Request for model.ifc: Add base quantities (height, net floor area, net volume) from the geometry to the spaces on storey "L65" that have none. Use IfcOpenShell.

First a look at what the model holds.

```python
import ifcopenshell
import ifcopenshell.util.element
import ifcopenshell.util.unit

model = ifcopenshell.open("model.ifc")
print(model.schema)
for unit_type in ("LENGTHUNIT", "AREAUNIT", "VOLUMEUNIT"):
    print(unit_type, ifcopenshell.util.unit.calculate_unit_scale(model, unit_type))
storey = next(s for s in model.by_type("IfcBuildingStorey") if s.Name == "L65")
spaces = [e for e in ifcopenshell.util.element.get_decomposition(storey) if e.is_a("IfcSpace")]
for e in sorted(spaces, key=lambda e: e.id()):
    print(e.id(), e.is_a(), e.Name, list(ifcopenshell.util.element.get_psets(e, qtos_only=True)), sep=" | ")
```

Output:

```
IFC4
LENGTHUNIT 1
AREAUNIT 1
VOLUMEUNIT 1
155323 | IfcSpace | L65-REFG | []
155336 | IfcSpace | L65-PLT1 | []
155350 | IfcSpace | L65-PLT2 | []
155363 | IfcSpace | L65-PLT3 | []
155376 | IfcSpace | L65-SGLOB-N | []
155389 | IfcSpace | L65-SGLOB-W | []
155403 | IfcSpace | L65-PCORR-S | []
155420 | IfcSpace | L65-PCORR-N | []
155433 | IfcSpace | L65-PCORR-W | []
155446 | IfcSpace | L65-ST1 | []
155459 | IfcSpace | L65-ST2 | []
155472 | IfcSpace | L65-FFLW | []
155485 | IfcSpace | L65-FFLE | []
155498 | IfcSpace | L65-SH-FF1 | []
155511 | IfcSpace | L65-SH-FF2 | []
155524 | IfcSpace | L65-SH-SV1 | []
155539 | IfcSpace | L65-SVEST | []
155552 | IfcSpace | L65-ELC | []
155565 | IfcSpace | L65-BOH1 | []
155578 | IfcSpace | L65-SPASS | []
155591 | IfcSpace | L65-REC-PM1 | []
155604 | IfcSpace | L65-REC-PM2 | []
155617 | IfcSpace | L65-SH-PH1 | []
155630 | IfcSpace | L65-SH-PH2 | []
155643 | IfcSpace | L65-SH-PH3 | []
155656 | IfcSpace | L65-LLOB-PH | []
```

```python
import ifcopenshell
import ifcopenshell.api.pset
import ifcopenshell.geom
import ifcopenshell.util.element
import ifcopenshell.util.shape
import ifcopenshell.util.unit

model = ifcopenshell.open("model.ifc")
unit_scale = ifcopenshell.util.unit.calculate_unit_scale(model)
area_scale = ifcopenshell.util.unit.calculate_unit_scale(model, "AREAUNIT")
volume_scale = ifcopenshell.util.unit.calculate_unit_scale(model, "VOLUMEUNIT")
settings = ifcopenshell.geom.settings()

storey = next(s for s in model.by_type("IfcBuildingStorey") if s.Name == "L65")
spaces = [e for e in ifcopenshell.util.element.get_decomposition(storey) if e.is_a("IfcSpace")]

for e in sorted(spaces, key=lambda e: e.id()):
    if ifcopenshell.util.element.get_psets(e, qtos_only=True, should_inherit=False):
        continue
    # Geometry comes back in metres, in the element's own axes.
    shape = ifcopenshell.geom.create_shape(settings, e)
    values = {
        "Height": ifcopenshell.util.shape.get_z(shape.geometry) / unit_scale,
        "NetFloorArea": ifcopenshell.util.shape.get_footprint_area(shape.geometry) / area_scale,
        "NetVolume": ifcopenshell.util.shape.get_volume(shape.geometry) / volume_scale,
    }
    qto = ifcopenshell.api.pset.add_qto(model, product=e, name="Qto_SpaceBaseQuantities")
    ifcopenshell.api.pset.edit_qto(model, qto=qto, properties=values)
    print(e.id(), {k: round(v, 3) for k, v in values.items()})

model.write("model-out.ifc")
```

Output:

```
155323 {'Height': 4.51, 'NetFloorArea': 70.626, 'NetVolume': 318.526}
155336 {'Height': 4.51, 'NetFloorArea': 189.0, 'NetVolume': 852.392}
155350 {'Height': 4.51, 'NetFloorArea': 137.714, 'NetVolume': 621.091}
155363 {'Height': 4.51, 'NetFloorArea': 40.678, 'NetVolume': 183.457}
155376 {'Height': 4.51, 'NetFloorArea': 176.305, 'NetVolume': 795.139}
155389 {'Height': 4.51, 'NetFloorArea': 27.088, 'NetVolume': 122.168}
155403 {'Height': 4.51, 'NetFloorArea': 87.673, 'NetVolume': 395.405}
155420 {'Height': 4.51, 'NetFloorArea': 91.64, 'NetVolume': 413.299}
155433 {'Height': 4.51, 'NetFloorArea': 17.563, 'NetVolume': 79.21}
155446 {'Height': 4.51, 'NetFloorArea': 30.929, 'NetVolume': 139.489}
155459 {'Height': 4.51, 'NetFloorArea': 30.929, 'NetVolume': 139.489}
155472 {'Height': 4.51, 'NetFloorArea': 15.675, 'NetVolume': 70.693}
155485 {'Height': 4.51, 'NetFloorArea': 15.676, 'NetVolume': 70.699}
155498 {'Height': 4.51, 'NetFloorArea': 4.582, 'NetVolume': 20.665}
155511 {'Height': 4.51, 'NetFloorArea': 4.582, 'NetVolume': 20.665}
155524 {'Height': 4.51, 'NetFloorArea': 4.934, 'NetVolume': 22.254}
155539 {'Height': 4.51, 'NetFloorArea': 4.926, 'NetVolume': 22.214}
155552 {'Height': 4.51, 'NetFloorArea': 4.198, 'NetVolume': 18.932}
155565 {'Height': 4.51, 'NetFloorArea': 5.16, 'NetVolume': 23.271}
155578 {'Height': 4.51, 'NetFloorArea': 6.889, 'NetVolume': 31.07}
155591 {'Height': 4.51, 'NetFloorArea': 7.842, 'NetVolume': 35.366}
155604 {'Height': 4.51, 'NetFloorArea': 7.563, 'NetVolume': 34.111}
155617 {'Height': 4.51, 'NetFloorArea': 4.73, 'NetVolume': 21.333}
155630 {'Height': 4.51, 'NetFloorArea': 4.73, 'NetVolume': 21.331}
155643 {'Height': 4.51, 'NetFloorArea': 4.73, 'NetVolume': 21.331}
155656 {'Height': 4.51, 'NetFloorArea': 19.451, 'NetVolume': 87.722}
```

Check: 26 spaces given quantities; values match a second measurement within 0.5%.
